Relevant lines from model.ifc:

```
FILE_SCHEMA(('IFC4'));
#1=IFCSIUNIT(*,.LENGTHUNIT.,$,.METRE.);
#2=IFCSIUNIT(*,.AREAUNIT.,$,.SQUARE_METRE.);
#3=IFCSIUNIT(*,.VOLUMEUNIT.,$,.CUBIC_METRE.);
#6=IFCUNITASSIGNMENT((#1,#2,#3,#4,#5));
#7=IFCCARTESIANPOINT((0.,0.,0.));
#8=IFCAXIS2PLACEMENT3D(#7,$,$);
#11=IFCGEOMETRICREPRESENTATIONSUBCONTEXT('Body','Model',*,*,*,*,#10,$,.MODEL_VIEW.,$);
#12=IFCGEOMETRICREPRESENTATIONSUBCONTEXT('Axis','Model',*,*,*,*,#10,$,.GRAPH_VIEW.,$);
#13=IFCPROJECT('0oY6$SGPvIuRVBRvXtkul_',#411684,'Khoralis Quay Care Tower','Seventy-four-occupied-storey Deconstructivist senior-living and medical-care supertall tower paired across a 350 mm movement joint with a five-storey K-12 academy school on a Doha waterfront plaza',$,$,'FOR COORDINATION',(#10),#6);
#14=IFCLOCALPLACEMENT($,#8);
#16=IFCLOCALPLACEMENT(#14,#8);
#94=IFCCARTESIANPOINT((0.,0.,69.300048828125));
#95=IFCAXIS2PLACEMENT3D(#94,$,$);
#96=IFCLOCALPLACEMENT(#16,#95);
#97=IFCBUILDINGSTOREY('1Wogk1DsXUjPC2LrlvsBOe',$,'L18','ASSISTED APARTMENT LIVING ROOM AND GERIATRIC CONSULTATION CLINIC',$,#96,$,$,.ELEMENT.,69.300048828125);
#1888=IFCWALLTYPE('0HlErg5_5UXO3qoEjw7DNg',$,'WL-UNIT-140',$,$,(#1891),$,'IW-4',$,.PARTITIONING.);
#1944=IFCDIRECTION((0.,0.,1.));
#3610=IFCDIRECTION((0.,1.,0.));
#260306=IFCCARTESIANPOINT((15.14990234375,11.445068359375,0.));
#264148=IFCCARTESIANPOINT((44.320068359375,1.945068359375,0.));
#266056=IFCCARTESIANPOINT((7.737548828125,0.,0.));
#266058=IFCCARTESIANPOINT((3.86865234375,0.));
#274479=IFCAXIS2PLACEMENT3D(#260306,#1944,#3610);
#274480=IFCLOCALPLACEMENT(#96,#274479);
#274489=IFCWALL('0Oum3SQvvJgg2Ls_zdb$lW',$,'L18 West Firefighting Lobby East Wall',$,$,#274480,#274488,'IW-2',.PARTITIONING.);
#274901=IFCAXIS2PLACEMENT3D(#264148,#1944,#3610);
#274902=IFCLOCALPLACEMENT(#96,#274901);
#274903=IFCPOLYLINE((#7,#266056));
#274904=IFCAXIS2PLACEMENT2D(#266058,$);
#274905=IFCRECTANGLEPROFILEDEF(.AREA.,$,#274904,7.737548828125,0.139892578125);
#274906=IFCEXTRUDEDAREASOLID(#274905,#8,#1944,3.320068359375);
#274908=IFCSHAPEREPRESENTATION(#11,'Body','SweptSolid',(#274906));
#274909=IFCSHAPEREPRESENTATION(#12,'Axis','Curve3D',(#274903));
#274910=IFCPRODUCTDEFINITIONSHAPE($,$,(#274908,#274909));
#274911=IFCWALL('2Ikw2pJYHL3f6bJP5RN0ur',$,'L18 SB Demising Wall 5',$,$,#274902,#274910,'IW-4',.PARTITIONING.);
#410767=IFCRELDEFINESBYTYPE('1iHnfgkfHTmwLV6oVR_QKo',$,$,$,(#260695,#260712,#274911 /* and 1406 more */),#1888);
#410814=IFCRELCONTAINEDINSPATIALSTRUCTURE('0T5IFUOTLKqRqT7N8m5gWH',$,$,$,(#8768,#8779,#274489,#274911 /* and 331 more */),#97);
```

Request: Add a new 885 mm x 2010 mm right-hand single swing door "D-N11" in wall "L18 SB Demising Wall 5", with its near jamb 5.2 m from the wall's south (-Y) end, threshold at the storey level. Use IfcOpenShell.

```python
import numpy as np
import ifcopenshell
import ifcopenshell.api.feature
import ifcopenshell.api.geometry
import ifcopenshell.api.root
import ifcopenshell.api.spatial
import ifcopenshell.geom
import ifcopenshell.util.element
import ifcopenshell.util.placement
import ifcopenshell.util.representation
import ifcopenshell.util.shape
import ifcopenshell.util.unit

model = ifcopenshell.open("model.ifc")
unit_scale = ifcopenshell.util.unit.calculate_unit_scale(model)
settings = ifcopenshell.geom.settings()


def volume(element):
    """Net volume in cubic metres, openings subtracted."""
    shape = ifcopenshell.geom.create_shape(settings, element)
    return ifcopenshell.util.shape.get_volume(shape.geometry)


wall = model.by_guid("2Ikw2pJYHL3f6bJP5RN0ur")
storey = ifcopenshell.util.element.get_container(wall, ifc_class="IfcBuildingStorey")
context = ifcopenshell.util.representation.get_context(model, "Model", "Body", "MODEL_VIEW")
before = volume(wall)

width, height, from_end, sill = 0.885, 2.01, 5.2, 0.0  # metres

# The wall runs along its own X axis, and the end named is its -X end.
wall_shape = ifcopenshell.geom.create_shape(settings, wall)
x, y, z = ifcopenshell.util.shape.get_vertices(wall_shape.geometry).T
start = x.min() + from_end
face, thickness = float(y.min()), float(y.max() - y.min())
wall_matrix = ifcopenshell.util.placement.get_local_placement(wall.ObjectPlacement)
level = ifcopenshell.util.placement.get_local_placement(storey.ObjectPlacement)[2, 3]


def in_wall(x, y):
    """Placement at x, y metres in the wall's axes, at sill height."""
    matrix = wall_matrix.copy()
    matrix[:, 3] = wall_matrix @ np.array([x / unit_scale, y / unit_scale, 0.0, 1.0])
    matrix[2, 3] = level + sill / unit_scale
    return matrix


# Opening: a box that overshoots both wall faces by 50 mm.
opening = ifcopenshell.api.root.create_entity(model, ifc_class="IfcOpeningElement", predefined_type="OPENING")
box = ifcopenshell.api.geometry.add_wall_representation(
    model, context=context, length=width, height=height, thickness=thickness + 0.1
)
ifcopenshell.api.geometry.assign_representation(model, product=opening, representation=box)
ifcopenshell.api.geometry.edit_object_placement(model, product=opening, matrix=in_wall(start, face - 0.05), is_si=False)
ifcopenshell.api.feature.add_feature(model, feature=opening, element=wall)

door = ifcopenshell.api.root.create_entity(model, ifc_class="IfcDoor", name="D-N11", predefined_type="DOOR")
door.OverallWidth, door.OverallHeight = width / unit_scale, height / unit_scale
door.OperationType = "SINGLE_SWING_RIGHT"
body = ifcopenshell.api.geometry.add_door_representation(
    model,
    context=context,
    overall_width=door.OverallWidth,
    overall_height=door.OverallHeight,
    operation_type="SINGLE_SWING_RIGHT",
    lining_properties={"LiningDepth": thickness / unit_scale, "ThresholdDepth": thickness / unit_scale},
)
ifcopenshell.api.geometry.assign_representation(model, product=door, representation=body)
ifcopenshell.api.spatial.assign_container(model, products=[door], relating_structure=storey)
ifcopenshell.api.feature.add_filling(model, opening=opening, element=door)

# The lining spans the wall, so the door starts at the wall face.
ifcopenshell.api.geometry.edit_object_placement(model, product=door, matrix=in_wall(start, face), is_si=False)

after = volume(wall)

print(f"wall volume {before:.3f} -> {after:.3f} m3")

model.write("model-out.ifc")
```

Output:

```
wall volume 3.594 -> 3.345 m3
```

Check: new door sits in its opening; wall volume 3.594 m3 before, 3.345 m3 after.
